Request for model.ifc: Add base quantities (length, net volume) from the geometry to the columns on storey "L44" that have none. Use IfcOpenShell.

First a look at what the model holds.

```python
import ifcopenshell
import ifcopenshell.util.element
import ifcopenshell.util.unit

model = ifcopenshell.open("model.ifc")
print(model.schema)
for unit_type in ("LENGTHUNIT", "AREAUNIT", "VOLUMEUNIT"):
    print(unit_type, ifcopenshell.util.unit.calculate_unit_scale(model, unit_type))
storey = next(s for s in model.by_type("IfcBuildingStorey") if s.Name == "L44")
columns = [e for e in ifcopenshell.util.element.get_decomposition(storey) if e.is_a("IfcColumn")]
for e in sorted(columns, key=lambda e: e.id()):
    print(e.id(), e.is_a(), e.Name, list(ifcopenshell.util.element.get_psets(e, qtos_only=True)), sep=" | ")
```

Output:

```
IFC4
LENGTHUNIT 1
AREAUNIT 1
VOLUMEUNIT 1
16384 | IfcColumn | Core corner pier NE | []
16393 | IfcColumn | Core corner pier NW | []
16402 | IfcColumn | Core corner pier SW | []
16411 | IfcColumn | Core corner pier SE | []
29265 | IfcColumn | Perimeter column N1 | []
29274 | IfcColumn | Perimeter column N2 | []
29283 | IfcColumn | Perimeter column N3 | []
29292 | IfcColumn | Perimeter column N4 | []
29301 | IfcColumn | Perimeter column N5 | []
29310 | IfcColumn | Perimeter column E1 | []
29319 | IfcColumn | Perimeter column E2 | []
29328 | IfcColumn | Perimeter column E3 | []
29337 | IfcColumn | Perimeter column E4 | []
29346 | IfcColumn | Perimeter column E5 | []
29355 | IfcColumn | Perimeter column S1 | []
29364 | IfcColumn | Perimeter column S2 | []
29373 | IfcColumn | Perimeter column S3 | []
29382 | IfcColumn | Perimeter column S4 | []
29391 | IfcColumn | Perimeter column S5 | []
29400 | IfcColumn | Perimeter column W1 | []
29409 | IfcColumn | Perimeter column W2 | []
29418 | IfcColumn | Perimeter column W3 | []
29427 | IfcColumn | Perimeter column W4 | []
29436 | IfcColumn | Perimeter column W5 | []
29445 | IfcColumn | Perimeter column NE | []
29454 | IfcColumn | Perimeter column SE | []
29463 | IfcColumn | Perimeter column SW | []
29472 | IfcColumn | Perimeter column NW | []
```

```python
import ifcopenshell
import ifcopenshell.api.pset
import ifcopenshell.geom
import ifcopenshell.util.element
import ifcopenshell.util.shape
import ifcopenshell.util.unit

model = ifcopenshell.open("model.ifc")
unit_scale = ifcopenshell.util.unit.calculate_unit_scale(model)
volume_scale = ifcopenshell.util.unit.calculate_unit_scale(model, "VOLUMEUNIT")
settings = ifcopenshell.geom.settings()

storey = next(s for s in model.by_type("IfcBuildingStorey") if s.Name == "L44")
columns = [e for e in ifcopenshell.util.element.get_decomposition(storey) if e.is_a("IfcColumn")]

for e in sorted(columns, key=lambda e: e.id()):
    if ifcopenshell.util.element.get_psets(e, qtos_only=True, should_inherit=False):
        continue
    # Geometry comes back in metres, in the element's own axes.
    shape = ifcopenshell.geom.create_shape(settings, e)
    values = {
        "Length": ifcopenshell.util.shape.get_z(shape.geometry) / unit_scale,
        "NetVolume": ifcopenshell.util.shape.get_volume(shape.geometry) / volume_scale,
    }
    qto = ifcopenshell.api.pset.add_qto(model, product=e, name="Qto_ColumnBaseQuantities")
    ifcopenshell.api.pset.edit_qto(model, qto=qto, properties=values)
    print(e.id(), {k: round(v, 3) for k, v in values.items()})

model.write("model_updated.ifc")
```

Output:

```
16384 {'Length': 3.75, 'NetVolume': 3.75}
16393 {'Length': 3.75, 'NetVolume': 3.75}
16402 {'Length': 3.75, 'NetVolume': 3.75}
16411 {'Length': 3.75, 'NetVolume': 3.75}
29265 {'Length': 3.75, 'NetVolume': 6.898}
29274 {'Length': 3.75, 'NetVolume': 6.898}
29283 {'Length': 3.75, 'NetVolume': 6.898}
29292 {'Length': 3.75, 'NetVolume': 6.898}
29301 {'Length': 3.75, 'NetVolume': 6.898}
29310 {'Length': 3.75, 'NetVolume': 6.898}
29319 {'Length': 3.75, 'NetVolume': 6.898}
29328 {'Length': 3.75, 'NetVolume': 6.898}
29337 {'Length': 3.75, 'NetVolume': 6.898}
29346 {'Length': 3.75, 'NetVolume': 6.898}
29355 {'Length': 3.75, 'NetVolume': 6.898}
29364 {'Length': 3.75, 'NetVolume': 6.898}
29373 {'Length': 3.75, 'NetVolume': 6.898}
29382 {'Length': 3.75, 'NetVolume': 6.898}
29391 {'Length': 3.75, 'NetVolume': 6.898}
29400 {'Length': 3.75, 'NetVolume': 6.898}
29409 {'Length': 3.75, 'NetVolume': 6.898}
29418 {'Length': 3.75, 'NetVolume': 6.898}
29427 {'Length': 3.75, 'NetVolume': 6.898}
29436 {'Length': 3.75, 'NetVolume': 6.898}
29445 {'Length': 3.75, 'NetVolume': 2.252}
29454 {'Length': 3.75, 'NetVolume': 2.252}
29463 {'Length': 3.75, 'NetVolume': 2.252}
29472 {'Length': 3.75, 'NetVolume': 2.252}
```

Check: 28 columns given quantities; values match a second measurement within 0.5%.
